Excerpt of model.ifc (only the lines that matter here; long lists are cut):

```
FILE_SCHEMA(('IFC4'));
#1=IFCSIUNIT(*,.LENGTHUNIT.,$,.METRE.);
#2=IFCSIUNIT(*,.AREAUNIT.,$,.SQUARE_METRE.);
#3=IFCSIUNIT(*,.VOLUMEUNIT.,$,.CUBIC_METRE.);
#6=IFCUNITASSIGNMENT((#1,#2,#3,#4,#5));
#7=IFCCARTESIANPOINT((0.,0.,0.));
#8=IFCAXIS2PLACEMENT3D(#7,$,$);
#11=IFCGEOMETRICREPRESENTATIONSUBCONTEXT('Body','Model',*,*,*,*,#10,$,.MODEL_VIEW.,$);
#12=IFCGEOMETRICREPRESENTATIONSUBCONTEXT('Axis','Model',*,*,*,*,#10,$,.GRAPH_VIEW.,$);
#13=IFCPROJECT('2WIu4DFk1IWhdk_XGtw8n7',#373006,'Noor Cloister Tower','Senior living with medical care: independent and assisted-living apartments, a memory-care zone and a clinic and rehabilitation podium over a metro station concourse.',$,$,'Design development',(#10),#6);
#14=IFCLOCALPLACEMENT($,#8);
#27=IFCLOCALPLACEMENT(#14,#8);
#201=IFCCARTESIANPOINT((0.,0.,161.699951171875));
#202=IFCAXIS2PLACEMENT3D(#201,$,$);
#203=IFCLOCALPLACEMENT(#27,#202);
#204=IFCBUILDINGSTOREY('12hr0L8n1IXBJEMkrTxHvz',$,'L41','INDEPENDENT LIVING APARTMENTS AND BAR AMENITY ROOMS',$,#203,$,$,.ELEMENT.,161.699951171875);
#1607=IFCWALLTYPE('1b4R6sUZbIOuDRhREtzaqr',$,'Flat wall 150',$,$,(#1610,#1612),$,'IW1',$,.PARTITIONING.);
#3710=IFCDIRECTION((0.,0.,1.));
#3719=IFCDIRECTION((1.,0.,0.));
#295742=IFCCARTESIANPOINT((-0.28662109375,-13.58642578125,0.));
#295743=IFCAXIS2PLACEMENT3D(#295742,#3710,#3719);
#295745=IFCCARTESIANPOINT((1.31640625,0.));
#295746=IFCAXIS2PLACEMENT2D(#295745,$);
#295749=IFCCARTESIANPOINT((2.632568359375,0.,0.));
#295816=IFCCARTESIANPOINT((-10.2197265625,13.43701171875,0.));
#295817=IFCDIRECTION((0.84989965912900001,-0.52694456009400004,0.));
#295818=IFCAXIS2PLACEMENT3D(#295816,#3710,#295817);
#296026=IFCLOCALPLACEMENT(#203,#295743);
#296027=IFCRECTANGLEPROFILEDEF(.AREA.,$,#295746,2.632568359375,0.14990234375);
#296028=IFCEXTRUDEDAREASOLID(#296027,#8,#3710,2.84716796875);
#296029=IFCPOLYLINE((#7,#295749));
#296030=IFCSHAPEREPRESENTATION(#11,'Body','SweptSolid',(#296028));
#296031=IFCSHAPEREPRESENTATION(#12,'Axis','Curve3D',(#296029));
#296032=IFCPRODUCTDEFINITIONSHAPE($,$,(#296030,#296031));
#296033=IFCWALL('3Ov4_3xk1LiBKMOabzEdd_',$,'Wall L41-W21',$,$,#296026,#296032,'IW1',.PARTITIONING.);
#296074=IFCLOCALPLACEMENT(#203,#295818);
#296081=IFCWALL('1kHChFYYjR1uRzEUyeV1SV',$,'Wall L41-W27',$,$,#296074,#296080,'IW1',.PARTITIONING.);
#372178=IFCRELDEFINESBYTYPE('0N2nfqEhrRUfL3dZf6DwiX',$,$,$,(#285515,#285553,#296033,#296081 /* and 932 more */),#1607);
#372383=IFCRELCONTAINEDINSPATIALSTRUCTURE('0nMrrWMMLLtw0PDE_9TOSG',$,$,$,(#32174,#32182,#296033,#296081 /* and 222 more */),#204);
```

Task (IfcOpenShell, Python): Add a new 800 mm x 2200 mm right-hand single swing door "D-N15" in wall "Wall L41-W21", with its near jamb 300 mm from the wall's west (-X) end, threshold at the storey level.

```python
import numpy as np
import ifcopenshell
import ifcopenshell.api.feature
import ifcopenshell.api.geometry
import ifcopenshell.api.root
import ifcopenshell.api.spatial
import ifcopenshell.geom
import ifcopenshell.util.element
import ifcopenshell.util.placement
import ifcopenshell.util.representation
import ifcopenshell.util.shape
import ifcopenshell.util.unit

model = ifcopenshell.open("model.ifc")
unit_scale = ifcopenshell.util.unit.calculate_unit_scale(model)
settings = ifcopenshell.geom.settings()


def volume(element):
    """Net volume in cubic metres, openings subtracted."""
    shape = ifcopenshell.geom.create_shape(settings, element)
    return ifcopenshell.util.shape.get_volume(shape.geometry)


wall = model.by_id(296033)
storey = ifcopenshell.util.element.get_container(wall, ifc_class="IfcBuildingStorey")
context = ifcopenshell.util.representation.get_context(model, "Model", "Body", "MODEL_VIEW")
before = volume(wall)

width, height, from_end, sill = 0.8, 2.2, 0.3, 0.0  # metres

# The wall runs along its own X axis, and the end named is its -X end.
wall_shape = ifcopenshell.geom.create_shape(settings, wall)
x, y, z = ifcopenshell.util.shape.get_vertices(wall_shape.geometry).T
start = x.min() + from_end
face, thickness = float(y.min()), float(y.max() - y.min())
wall_matrix = ifcopenshell.util.placement.get_local_placement(wall.ObjectPlacement)
level = ifcopenshell.util.placement.get_local_placement(storey.ObjectPlacement)[2, 3]


def in_wall(x, y):
    """Placement at x, y metres in the wall's axes, at sill height."""
    matrix = wall_matrix.copy()
    matrix[:, 3] = wall_matrix @ np.array([x / unit_scale, y / unit_scale, 0.0, 1.0])
    matrix[2, 3] = level + sill / unit_scale
    return matrix


# Opening: a box that overshoots both wall faces by 50 mm.
opening = ifcopenshell.api.root.create_entity(model, ifc_class="IfcOpeningElement", predefined_type="OPENING")
box = ifcopenshell.api.geometry.add_wall_representation(
    model, context=context, length=width, height=height, thickness=thickness + 0.1
)
ifcopenshell.api.geometry.assign_representation(model, product=opening, representation=box)
ifcopenshell.api.geometry.edit_object_placement(model, product=opening, matrix=in_wall(start, face - 0.05), is_si=False)
ifcopenshell.api.feature.add_feature(model, feature=opening, element=wall)

door = ifcopenshell.api.root.create_entity(model, ifc_class="IfcDoor", name="D-N15", predefined_type="DOOR")
door.OverallWidth, door.OverallHeight = width / unit_scale, height / unit_scale
door.OperationType = "SINGLE_SWING_RIGHT"
body = ifcopenshell.api.geometry.add_door_representation(
    model,
    context=context,
    overall_width=door.OverallWidth,
    overall_height=door.OverallHeight,
    operation_type="SINGLE_SWING_RIGHT",
    lining_properties={"LiningDepth": thickness / unit_scale, "ThresholdDepth": thickness / unit_scale},
)
ifcopenshell.api.geometry.assign_representation(model, product=door, representation=body)
ifcopenshell.api.spatial.assign_container(model, products=[door], relating_structure=storey)
ifcopenshell.api.feature.add_filling(model, opening=opening, element=door)

# The lining spans the wall, so the door starts at the wall face.
ifcopenshell.api.geometry.edit_object_placement(model, product=door, matrix=in_wall(start, face), is_si=False)

after = volume(wall)

print(f"wall volume {before:.3f} -> {after:.3f} m3")

model.write("model_updated.ifc")
```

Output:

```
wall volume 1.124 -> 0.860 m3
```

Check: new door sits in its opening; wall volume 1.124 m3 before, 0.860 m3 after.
